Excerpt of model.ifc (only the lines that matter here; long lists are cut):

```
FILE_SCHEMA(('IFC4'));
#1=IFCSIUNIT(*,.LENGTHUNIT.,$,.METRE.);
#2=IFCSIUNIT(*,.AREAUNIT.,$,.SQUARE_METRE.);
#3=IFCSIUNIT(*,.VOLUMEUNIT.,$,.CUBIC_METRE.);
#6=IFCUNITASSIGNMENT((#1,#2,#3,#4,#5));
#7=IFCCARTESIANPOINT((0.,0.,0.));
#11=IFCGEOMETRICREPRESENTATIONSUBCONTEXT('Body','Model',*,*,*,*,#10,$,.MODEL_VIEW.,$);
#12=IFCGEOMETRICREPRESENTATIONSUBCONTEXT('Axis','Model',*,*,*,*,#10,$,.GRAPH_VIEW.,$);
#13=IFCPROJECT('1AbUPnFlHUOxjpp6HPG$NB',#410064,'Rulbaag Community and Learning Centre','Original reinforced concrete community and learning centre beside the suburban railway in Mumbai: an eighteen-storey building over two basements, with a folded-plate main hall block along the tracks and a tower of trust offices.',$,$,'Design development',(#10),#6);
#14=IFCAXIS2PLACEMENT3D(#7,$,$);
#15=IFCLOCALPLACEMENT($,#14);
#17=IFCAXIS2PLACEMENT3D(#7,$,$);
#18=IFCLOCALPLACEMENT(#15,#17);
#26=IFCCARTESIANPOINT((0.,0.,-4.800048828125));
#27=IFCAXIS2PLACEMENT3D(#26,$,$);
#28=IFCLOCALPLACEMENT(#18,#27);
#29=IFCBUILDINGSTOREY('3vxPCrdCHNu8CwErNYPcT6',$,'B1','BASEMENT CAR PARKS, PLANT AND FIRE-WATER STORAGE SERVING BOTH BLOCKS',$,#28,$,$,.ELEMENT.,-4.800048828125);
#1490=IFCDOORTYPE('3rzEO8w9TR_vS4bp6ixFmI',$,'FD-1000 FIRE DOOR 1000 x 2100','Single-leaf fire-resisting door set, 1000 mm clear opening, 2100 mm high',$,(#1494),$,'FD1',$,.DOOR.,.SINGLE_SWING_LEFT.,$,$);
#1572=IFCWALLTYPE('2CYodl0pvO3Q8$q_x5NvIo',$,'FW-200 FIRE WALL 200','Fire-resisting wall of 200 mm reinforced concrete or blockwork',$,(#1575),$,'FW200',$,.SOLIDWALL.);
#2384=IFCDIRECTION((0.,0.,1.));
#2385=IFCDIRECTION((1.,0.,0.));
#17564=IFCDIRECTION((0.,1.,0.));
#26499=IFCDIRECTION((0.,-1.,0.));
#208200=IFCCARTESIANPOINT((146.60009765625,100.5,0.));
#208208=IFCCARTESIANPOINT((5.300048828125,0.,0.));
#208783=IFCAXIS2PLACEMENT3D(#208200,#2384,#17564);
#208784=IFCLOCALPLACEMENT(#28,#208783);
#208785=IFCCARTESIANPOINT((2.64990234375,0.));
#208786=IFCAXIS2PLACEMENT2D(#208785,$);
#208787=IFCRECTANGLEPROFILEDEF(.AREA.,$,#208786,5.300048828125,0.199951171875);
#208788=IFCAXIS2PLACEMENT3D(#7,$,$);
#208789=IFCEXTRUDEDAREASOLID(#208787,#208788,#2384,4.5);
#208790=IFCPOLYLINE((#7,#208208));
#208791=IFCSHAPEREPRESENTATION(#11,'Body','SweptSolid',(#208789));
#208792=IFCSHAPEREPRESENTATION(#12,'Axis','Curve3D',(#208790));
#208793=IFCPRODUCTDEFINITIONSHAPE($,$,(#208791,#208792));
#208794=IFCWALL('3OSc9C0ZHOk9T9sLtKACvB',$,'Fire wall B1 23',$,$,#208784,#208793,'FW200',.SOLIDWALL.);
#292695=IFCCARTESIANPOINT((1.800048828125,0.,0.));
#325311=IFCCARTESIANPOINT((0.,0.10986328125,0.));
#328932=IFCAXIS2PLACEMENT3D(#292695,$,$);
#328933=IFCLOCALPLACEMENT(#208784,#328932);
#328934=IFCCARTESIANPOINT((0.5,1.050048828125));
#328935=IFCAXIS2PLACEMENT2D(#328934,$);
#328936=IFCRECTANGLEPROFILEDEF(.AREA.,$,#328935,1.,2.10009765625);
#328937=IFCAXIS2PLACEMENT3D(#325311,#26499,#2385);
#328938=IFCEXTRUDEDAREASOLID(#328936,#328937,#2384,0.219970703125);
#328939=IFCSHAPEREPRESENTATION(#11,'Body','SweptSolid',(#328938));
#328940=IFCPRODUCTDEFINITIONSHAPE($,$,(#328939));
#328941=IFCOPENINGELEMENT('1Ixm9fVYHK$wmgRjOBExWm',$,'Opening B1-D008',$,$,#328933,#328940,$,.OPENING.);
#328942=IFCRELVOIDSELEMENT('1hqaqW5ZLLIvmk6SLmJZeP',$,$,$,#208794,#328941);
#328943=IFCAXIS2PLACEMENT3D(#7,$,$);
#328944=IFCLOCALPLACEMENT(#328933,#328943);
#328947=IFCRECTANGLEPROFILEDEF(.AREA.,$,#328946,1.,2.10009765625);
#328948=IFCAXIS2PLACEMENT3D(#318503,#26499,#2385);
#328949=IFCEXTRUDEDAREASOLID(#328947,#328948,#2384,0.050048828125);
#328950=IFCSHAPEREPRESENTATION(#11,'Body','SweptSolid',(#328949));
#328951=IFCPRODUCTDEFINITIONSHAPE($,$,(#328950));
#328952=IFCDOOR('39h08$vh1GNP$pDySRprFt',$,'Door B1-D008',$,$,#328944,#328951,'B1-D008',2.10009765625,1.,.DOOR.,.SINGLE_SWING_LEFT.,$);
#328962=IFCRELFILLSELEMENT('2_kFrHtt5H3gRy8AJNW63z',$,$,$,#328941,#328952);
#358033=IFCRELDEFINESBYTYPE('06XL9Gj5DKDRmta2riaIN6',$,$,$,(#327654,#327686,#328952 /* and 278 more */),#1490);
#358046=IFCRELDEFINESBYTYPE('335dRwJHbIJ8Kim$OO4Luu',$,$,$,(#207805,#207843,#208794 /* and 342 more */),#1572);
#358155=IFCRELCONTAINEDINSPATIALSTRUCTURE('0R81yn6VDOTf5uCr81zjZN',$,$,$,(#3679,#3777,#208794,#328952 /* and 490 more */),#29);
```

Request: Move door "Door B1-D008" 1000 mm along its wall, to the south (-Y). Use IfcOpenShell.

```python
import ifcopenshell
import ifcopenshell.api.geometry
import ifcopenshell.util.placement

model = ifcopenshell.open("model.ifc")

door = model.by_guid("39h08$vh1GNP$pDySRprFt")
opening = door.FillsVoids[0].RelatingOpeningElement
wall = opening.VoidsElements[0].RelatingBuildingElement

wall_matrix = ifcopenshell.util.placement.get_local_placement(wall.ObjectPlacement)
shift = wall_matrix[:3, 0] * -1.0
before = ifcopenshell.util.placement.get_local_placement(door.ObjectPlacement)[:3, 3].copy()

# The door is placed relative to its opening, so it follows when the opening moves.
matrix = ifcopenshell.util.placement.get_local_placement(opening.ObjectPlacement)
matrix[:3, 3] += shift
ifcopenshell.api.geometry.edit_object_placement(
    model, product=opening, matrix=matrix, is_si=False, should_transform_children=True
)

after = ifcopenshell.util.placement.get_local_placement(door.ObjectPlacement)[:3, 3]
print("door moved by", (after - before).round(3) + 0.0)

model.write("model_v2.ifc")
```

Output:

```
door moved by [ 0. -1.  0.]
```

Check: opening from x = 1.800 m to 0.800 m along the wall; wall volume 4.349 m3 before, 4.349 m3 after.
